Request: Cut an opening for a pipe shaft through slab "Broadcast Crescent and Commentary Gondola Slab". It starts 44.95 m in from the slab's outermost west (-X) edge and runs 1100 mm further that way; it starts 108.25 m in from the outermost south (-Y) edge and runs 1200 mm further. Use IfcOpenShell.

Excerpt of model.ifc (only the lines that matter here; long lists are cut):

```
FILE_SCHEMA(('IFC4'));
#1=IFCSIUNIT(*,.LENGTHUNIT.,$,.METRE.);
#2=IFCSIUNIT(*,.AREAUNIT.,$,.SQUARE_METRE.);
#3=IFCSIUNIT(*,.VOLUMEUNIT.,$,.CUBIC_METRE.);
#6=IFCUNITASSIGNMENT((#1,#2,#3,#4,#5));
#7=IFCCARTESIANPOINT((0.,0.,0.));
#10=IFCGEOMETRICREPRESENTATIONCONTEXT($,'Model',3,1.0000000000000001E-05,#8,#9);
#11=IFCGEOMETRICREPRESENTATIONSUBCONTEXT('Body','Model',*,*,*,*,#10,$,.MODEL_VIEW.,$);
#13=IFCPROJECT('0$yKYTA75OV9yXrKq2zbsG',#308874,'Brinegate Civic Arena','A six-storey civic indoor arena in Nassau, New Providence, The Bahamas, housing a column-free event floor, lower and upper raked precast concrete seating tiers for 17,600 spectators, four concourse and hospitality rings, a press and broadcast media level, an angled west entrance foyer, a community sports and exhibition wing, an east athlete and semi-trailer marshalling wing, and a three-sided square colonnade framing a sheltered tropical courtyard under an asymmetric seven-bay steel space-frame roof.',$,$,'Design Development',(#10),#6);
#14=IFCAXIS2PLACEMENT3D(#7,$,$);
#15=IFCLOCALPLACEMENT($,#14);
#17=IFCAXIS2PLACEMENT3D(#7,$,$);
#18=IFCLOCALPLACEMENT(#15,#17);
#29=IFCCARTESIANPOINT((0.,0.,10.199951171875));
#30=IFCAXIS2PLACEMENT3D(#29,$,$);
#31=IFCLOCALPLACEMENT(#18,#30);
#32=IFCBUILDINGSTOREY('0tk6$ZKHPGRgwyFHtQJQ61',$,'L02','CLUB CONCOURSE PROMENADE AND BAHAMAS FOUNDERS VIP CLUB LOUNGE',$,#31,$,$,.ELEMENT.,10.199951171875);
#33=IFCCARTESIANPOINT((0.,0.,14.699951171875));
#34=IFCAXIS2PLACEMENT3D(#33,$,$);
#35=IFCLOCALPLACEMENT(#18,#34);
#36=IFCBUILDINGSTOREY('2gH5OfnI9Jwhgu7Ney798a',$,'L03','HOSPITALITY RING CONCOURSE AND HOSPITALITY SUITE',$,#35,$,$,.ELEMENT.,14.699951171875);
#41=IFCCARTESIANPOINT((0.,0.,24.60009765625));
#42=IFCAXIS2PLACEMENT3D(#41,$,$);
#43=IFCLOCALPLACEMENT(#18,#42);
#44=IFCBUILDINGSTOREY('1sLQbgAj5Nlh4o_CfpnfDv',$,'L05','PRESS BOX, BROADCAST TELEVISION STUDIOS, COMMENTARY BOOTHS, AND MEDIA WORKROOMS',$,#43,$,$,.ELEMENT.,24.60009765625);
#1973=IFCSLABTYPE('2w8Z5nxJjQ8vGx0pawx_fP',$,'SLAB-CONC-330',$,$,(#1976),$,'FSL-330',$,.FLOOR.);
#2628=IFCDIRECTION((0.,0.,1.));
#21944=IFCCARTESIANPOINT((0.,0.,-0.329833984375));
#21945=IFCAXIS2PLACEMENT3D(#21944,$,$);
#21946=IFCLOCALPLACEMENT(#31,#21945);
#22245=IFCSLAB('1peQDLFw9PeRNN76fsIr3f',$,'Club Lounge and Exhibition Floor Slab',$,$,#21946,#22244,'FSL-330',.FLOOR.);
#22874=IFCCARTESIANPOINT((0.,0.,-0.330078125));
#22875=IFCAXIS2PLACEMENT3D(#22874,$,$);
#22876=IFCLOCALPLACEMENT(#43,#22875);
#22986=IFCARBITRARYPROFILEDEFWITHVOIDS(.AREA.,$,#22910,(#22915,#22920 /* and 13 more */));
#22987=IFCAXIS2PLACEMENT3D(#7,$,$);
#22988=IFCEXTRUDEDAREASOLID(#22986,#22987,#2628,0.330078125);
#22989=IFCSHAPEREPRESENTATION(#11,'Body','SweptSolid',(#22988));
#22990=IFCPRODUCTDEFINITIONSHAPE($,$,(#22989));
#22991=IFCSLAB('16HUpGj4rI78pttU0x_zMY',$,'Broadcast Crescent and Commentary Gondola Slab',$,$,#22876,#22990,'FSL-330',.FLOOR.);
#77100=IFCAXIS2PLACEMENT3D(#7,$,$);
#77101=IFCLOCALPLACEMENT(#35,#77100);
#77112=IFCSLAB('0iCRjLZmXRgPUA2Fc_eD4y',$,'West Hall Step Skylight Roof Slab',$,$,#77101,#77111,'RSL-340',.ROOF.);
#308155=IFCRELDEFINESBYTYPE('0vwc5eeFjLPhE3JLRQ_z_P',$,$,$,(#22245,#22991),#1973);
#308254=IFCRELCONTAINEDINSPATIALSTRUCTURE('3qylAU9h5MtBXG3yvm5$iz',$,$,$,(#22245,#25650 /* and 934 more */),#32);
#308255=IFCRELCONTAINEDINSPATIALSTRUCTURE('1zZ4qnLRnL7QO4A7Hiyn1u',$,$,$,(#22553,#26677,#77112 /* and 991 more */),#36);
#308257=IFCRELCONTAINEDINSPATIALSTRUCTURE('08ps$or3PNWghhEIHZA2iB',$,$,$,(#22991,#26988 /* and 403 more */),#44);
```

```python
import numpy as np
import ifcopenshell
import ifcopenshell.api.feature
import ifcopenshell.api.geometry
import ifcopenshell.api.root
import ifcopenshell.geom
import ifcopenshell.util.placement
import ifcopenshell.util.representation
import ifcopenshell.util.shape
import ifcopenshell.util.unit

model = ifcopenshell.open("model.ifc")
unit_scale = ifcopenshell.util.unit.calculate_unit_scale(model)
settings = ifcopenshell.geom.settings()


def volume(element):
    """Net volume in cubic metres, openings subtracted."""
    shape = ifcopenshell.geom.create_shape(settings, element)
    return ifcopenshell.util.shape.get_volume(shape.geometry)


slab = model.by_guid("16HUpGj4rI78pttU0x_zMY")
before = volume(slab)

# Extent in the slab's own axes, in metres. The edges named are its -X and -Y sides.
slab_shape = ifcopenshell.geom.create_shape(settings, slab)
vertices = ifcopenshell.util.shape.get_vertices(slab_shape.geometry)
x_min, y_min, bottom = vertices.min(axis=0)
top = vertices[:, 2].max()

opening = ifcopenshell.api.root.create_entity(model, ifc_class="IfcOpeningElement", name="Pipe shaft opening", predefined_type="OPENING")
context = ifcopenshell.util.representation.get_context(model, "Model", "Body", "MODEL_VIEW")
width, depth = 1.1, 1.2
outline = [(0.0, 0.0), (width, 0.0), (width, depth), (0.0, depth), (0.0, 0.0)]
# Overshoot both faces by 50 mm so the cut is clean.
shape = ifcopenshell.api.geometry.add_slab_representation(
    model, context=context, depth=top - bottom + 0.1, polyline=outline
)
ifcopenshell.api.geometry.assign_representation(model, product=opening, representation=shape)

matrix = ifcopenshell.util.placement.get_local_placement(slab.ObjectPlacement)
matrix[:, 3] = matrix @ np.append(np.array([x_min + 44.95, y_min + 108.25, bottom - 0.05]) / unit_scale, 1.0)
ifcopenshell.api.geometry.edit_object_placement(model, product=opening, matrix=matrix, is_si=False)
ifcopenshell.api.feature.add_feature(model, feature=opening, element=slab)

after = volume(slab)

print(f"slab volume {before:.3f} -> {after:.3f} m3")

model.write("model_v2.ifc")
```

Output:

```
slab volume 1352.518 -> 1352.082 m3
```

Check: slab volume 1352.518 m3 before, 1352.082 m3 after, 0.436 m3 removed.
